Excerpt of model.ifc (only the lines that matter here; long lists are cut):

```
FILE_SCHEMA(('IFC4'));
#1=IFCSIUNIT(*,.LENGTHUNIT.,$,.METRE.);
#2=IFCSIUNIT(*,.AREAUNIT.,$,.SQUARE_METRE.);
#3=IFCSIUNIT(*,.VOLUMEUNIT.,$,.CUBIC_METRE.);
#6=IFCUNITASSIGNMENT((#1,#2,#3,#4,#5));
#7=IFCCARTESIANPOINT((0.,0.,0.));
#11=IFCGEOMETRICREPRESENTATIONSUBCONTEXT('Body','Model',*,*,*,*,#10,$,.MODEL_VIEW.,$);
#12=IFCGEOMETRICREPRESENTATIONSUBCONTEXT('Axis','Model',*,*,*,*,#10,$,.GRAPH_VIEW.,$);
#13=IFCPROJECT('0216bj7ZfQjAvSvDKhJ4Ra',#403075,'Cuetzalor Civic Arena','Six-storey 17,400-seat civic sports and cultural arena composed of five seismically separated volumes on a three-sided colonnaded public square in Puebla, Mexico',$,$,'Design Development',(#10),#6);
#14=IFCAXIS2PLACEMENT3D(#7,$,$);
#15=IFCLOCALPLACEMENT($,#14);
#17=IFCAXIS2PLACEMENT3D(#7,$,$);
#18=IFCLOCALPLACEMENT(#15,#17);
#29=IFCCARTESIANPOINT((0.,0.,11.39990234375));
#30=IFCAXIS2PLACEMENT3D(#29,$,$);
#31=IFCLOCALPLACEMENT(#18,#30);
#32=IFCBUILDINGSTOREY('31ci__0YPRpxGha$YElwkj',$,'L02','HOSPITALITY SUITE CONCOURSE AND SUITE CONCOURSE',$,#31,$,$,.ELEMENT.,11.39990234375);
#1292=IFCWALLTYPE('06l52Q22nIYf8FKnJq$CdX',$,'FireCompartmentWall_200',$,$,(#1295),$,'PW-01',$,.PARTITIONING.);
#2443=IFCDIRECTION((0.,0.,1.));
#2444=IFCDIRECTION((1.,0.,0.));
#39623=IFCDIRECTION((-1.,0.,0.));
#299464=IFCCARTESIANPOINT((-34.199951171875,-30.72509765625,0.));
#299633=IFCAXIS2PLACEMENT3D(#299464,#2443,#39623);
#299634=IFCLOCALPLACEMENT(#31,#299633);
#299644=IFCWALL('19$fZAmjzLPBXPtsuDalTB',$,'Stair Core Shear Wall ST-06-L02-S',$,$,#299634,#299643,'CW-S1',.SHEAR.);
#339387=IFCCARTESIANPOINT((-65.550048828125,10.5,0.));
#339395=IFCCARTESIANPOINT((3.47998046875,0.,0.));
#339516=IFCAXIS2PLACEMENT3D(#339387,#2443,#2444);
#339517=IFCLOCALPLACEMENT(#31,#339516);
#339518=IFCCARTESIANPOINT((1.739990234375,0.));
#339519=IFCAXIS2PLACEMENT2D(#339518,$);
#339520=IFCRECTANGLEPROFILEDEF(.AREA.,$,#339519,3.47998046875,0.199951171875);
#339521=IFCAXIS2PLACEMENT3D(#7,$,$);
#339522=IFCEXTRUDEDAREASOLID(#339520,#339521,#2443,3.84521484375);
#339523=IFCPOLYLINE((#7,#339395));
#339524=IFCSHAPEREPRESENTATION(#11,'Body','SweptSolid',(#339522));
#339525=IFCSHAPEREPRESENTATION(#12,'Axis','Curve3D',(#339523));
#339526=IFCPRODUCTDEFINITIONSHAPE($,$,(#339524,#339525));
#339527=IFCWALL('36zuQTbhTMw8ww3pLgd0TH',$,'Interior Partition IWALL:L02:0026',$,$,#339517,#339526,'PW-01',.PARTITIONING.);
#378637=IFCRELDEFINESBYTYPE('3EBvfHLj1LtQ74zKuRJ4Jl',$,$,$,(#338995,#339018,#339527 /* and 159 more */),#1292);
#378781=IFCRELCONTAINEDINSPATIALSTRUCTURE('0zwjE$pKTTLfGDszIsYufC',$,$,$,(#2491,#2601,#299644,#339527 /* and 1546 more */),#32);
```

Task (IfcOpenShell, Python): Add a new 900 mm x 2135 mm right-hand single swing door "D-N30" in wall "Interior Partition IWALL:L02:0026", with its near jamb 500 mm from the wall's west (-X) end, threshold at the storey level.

```python
import numpy as np
import ifcopenshell
import ifcopenshell.api.feature
import ifcopenshell.api.geometry
import ifcopenshell.api.root
import ifcopenshell.api.spatial
import ifcopenshell.geom
import ifcopenshell.util.element
import ifcopenshell.util.placement
import ifcopenshell.util.representation
import ifcopenshell.util.shape
import ifcopenshell.util.unit

model = ifcopenshell.open("model.ifc")
unit_scale = ifcopenshell.util.unit.calculate_unit_scale(model)
settings = ifcopenshell.geom.settings()


def volume(element):
    """Net volume in cubic metres, openings subtracted."""
    shape = ifcopenshell.geom.create_shape(settings, element)
    return ifcopenshell.util.shape.get_volume(shape.geometry)


wall = model.by_guid("36zuQTbhTMw8ww3pLgd0TH")
storey = ifcopenshell.util.element.get_container(wall, ifc_class="IfcBuildingStorey")
context = ifcopenshell.util.representation.get_context(model, "Model", "Body", "MODEL_VIEW")
before = volume(wall)

width, height, from_end, sill = 0.9, 2.135, 0.5, 0.0  # metres

# The wall runs along its own X axis, and the end named is its -X end.
wall_shape = ifcopenshell.geom.create_shape(settings, wall)
x, y, z = ifcopenshell.util.shape.get_vertices(wall_shape.geometry).T
start = x.min() + from_end
face, thickness = float(y.min()), float(y.max() - y.min())
wall_matrix = ifcopenshell.util.placement.get_local_placement(wall.ObjectPlacement)
level = ifcopenshell.util.placement.get_local_placement(storey.ObjectPlacement)[2, 3]


def in_wall(x, y):
    """Placement at x, y metres in the wall's axes, at sill height."""
    matrix = wall_matrix.copy()
    matrix[:, 3] = wall_matrix @ np.array([x / unit_scale, y / unit_scale, 0.0, 1.0])
    matrix[2, 3] = level + sill / unit_scale
    return matrix


# Opening: a box that overshoots both wall faces by 50 mm.
opening = ifcopenshell.api.root.create_entity(model, ifc_class="IfcOpeningElement", predefined_type="OPENING")
box = ifcopenshell.api.geometry.add_wall_representation(
    model, context=context, length=width, height=height, thickness=thickness + 0.1
)
ifcopenshell.api.geometry.assign_representation(model, product=opening, representation=box)
ifcopenshell.api.geometry.edit_object_placement(model, product=opening, matrix=in_wall(start, face - 0.05), is_si=False)
ifcopenshell.api.feature.add_feature(model, feature=opening, element=wall)

door = ifcopenshell.api.root.create_entity(model, ifc_class="IfcDoor", name="D-N30", predefined_type="DOOR")
door.OverallWidth, door.OverallHeight = width / unit_scale, height / unit_scale
door.OperationType = "SINGLE_SWING_RIGHT"
body = ifcopenshell.api.geometry.add_door_representation(
    model,
    context=context,
    overall_width=door.OverallWidth,
    overall_height=door.OverallHeight,
    operation_type="SINGLE_SWING_RIGHT",
    lining_properties={"LiningDepth": thickness / unit_scale, "ThresholdDepth": thickness / unit_scale},
)
ifcopenshell.api.geometry.assign_representation(model, product=door, representation=body)
ifcopenshell.api.spatial.assign_container(model, products=[door], relating_structure=storey)
ifcopenshell.api.feature.add_filling(model, opening=opening, element=door)

# The lining spans the wall, so the door starts at the wall face.
ifcopenshell.api.geometry.edit_object_placement(model, product=door, matrix=in_wall(start, face), is_si=False)

after = volume(wall)

print(f"wall volume {before:.3f} -> {after:.3f} m3")

model.write("model-out.ifc")
```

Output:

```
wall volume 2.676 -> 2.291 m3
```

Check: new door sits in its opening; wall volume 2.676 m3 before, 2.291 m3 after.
